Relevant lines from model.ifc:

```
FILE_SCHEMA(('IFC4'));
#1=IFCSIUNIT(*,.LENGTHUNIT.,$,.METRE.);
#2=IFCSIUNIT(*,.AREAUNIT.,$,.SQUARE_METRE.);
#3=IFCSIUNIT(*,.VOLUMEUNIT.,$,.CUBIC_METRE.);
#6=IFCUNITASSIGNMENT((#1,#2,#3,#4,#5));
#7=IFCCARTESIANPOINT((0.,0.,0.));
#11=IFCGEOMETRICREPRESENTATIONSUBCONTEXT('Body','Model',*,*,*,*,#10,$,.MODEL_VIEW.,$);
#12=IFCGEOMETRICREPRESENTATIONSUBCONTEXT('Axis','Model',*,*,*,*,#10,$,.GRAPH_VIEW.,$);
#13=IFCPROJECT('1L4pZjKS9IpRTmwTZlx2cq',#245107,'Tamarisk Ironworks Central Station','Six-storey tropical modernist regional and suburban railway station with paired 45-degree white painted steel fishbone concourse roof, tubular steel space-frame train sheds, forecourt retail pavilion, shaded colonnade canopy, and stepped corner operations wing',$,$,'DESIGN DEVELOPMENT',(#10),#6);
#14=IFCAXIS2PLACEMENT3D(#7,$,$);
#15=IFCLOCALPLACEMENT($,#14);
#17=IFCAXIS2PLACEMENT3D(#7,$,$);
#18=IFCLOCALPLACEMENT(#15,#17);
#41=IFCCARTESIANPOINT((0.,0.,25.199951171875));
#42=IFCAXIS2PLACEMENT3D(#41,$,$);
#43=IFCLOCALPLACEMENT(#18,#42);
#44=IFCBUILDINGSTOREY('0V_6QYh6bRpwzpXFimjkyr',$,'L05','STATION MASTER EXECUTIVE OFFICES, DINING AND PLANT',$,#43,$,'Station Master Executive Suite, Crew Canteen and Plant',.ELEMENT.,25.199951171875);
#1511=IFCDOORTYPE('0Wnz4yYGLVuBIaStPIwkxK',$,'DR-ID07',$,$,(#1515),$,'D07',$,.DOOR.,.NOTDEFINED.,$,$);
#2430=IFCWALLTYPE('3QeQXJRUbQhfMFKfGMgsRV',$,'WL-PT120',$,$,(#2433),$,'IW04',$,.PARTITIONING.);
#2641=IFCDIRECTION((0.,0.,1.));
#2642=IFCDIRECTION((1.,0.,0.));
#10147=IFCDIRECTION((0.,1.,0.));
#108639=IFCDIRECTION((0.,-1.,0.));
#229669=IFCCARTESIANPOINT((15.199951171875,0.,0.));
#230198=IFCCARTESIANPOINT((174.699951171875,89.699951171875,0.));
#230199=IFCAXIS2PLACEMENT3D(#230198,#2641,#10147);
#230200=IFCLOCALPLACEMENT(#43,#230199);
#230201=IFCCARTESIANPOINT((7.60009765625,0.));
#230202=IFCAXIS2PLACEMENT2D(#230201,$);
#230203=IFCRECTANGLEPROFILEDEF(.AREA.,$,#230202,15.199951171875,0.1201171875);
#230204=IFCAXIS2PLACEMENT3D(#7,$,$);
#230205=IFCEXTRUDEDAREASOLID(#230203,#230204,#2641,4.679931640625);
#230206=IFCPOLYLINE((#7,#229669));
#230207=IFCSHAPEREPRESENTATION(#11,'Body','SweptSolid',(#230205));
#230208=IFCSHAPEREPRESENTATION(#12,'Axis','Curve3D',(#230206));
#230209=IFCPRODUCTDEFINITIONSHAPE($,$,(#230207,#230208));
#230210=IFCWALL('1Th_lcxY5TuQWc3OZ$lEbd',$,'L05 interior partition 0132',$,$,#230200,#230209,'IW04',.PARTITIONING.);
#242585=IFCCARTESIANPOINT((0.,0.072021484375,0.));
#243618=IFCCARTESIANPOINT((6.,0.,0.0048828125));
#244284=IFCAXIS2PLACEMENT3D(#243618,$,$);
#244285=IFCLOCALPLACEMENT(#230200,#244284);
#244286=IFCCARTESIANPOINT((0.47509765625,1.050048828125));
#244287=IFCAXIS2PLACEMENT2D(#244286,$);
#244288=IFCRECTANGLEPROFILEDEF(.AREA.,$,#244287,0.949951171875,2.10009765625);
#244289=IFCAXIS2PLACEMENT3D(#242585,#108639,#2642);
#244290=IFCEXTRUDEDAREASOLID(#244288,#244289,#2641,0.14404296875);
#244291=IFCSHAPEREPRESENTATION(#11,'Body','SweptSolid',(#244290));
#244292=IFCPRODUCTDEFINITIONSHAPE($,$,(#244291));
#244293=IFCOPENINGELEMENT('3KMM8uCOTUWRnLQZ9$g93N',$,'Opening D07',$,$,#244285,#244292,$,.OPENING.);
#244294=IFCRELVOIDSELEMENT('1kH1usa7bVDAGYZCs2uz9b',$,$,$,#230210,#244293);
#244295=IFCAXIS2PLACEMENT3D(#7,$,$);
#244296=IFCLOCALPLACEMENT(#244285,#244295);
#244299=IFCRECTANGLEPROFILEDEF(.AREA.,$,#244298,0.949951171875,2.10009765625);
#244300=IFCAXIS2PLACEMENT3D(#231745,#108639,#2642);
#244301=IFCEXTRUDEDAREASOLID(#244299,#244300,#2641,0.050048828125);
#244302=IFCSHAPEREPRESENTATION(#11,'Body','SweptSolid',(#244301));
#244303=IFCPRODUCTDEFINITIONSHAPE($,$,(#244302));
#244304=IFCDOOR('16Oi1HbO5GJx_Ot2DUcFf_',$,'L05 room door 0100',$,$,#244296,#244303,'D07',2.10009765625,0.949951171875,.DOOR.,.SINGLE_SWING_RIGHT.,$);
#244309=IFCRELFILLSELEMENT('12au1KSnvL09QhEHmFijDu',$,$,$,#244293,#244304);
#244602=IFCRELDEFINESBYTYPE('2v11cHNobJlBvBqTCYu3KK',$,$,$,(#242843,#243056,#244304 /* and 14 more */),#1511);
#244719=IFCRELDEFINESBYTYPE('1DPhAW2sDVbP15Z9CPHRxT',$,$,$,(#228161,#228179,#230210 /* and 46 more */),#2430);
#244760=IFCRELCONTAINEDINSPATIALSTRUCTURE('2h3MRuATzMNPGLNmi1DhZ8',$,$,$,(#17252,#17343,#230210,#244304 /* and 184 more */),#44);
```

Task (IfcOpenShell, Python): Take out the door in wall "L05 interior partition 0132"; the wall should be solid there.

```python
import ifcopenshell
import ifcopenshell.api.feature
import ifcopenshell.api.root
import ifcopenshell.geom
import ifcopenshell.util.shape

model = ifcopenshell.open("model.ifc")
settings = ifcopenshell.geom.settings()


def volume(element):
    """Net volume in cubic metres, openings subtracted."""
    shape = ifcopenshell.geom.create_shape(settings, element)
    return ifcopenshell.util.shape.get_volume(shape.geometry)


door = model.by_id(244304)
opening = door.FillsVoids[0].RelatingOpeningElement
wall = opening.VoidsElements[0].RelatingBuildingElement
before = volume(wall)

ifcopenshell.api.root.remove_product(model, product=door)
ifcopenshell.api.feature.remove_feature(model, feature=opening)

after = volume(wall)

print(f"wall volume {before:.3f} -> {after:.3f} m3")

model.write("model_updated.ifc")
```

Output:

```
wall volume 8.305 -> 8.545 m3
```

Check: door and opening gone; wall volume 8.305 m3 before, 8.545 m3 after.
